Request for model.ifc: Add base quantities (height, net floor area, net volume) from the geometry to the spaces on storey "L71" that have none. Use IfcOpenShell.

First a look at what the model holds.

```python
import ifcopenshell
import ifcopenshell.util.element
import ifcopenshell.util.unit

model = ifcopenshell.open("model.ifc")
print(model.schema)
for unit_type in ("LENGTHUNIT", "AREAUNIT", "VOLUMEUNIT"):
    print(unit_type, ifcopenshell.util.unit.calculate_unit_scale(model, unit_type))
storey = next(s for s in model.by_type("IfcBuildingStorey") if s.Name == "L71")
spaces = [e for e in ifcopenshell.util.element.get_decomposition(storey) if e.is_a("IfcSpace")]
for e in sorted(spaces, key=lambda e: e.id()):
    print(e.id(), e.is_a(), e.Name, list(ifcopenshell.util.element.get_psets(e, qtos_only=True)), sep=" | ")
```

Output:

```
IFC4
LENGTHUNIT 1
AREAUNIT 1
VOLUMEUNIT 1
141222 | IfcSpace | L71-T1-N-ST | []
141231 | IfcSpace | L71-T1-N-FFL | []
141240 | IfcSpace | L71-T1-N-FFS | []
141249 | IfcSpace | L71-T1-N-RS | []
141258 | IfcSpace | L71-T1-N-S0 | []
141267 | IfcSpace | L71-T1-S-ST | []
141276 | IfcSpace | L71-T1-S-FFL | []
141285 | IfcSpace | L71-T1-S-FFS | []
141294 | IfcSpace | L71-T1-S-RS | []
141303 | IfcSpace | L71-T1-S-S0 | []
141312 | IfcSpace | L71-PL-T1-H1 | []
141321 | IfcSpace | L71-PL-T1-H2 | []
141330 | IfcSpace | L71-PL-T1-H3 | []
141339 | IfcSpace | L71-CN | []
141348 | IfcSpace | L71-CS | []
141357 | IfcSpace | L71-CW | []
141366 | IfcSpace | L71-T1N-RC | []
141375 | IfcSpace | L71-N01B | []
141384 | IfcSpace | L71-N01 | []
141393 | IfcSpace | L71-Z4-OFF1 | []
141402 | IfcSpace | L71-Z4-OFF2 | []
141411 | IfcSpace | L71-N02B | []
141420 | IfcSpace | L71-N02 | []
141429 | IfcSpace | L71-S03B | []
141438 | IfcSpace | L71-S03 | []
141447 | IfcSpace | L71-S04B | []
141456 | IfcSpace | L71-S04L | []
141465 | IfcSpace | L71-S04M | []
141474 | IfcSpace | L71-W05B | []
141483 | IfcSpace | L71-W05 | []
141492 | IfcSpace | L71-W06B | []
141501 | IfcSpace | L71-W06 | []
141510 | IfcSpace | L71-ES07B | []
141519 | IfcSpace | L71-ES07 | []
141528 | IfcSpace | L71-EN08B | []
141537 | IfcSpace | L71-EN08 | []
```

```python
import ifcopenshell
import ifcopenshell.api.pset
import ifcopenshell.geom
import ifcopenshell.util.element
import ifcopenshell.util.shape
import ifcopenshell.util.unit

model = ifcopenshell.open("model.ifc")
unit_scale = ifcopenshell.util.unit.calculate_unit_scale(model)
area_scale = ifcopenshell.util.unit.calculate_unit_scale(model, "AREAUNIT")
volume_scale = ifcopenshell.util.unit.calculate_unit_scale(model, "VOLUMEUNIT")
settings = ifcopenshell.geom.settings()

storey = next(s for s in model.by_type("IfcBuildingStorey") if s.Name == "L71")
spaces = [e for e in ifcopenshell.util.element.get_decomposition(storey) if e.is_a("IfcSpace")]

for e in sorted(spaces, key=lambda e: e.id()):
    if ifcopenshell.util.element.get_psets(e, qtos_only=True, should_inherit=False):
        continue
    # Geometry comes back in metres, in the element's own axes.
    shape = ifcopenshell.geom.create_shape(settings, e)
    values = {
        "Height": ifcopenshell.util.shape.get_z(shape.geometry) / unit_scale,
        "NetFloorArea": ifcopenshell.util.shape.get_footprint_area(shape.geometry) / area_scale,
        "NetVolume": ifcopenshell.util.shape.get_volume(shape.geometry) / volume_scale,
    }
    qto = ifcopenshell.api.pset.add_qto(model, product=e, name="Qto_SpaceBaseQuantities")
    ifcopenshell.api.pset.edit_qto(model, qto=qto, properties=values)
    print(e.id(), {k: round(v, 3) for k, v in values.items()})

model.write("model_v2.ifc")
```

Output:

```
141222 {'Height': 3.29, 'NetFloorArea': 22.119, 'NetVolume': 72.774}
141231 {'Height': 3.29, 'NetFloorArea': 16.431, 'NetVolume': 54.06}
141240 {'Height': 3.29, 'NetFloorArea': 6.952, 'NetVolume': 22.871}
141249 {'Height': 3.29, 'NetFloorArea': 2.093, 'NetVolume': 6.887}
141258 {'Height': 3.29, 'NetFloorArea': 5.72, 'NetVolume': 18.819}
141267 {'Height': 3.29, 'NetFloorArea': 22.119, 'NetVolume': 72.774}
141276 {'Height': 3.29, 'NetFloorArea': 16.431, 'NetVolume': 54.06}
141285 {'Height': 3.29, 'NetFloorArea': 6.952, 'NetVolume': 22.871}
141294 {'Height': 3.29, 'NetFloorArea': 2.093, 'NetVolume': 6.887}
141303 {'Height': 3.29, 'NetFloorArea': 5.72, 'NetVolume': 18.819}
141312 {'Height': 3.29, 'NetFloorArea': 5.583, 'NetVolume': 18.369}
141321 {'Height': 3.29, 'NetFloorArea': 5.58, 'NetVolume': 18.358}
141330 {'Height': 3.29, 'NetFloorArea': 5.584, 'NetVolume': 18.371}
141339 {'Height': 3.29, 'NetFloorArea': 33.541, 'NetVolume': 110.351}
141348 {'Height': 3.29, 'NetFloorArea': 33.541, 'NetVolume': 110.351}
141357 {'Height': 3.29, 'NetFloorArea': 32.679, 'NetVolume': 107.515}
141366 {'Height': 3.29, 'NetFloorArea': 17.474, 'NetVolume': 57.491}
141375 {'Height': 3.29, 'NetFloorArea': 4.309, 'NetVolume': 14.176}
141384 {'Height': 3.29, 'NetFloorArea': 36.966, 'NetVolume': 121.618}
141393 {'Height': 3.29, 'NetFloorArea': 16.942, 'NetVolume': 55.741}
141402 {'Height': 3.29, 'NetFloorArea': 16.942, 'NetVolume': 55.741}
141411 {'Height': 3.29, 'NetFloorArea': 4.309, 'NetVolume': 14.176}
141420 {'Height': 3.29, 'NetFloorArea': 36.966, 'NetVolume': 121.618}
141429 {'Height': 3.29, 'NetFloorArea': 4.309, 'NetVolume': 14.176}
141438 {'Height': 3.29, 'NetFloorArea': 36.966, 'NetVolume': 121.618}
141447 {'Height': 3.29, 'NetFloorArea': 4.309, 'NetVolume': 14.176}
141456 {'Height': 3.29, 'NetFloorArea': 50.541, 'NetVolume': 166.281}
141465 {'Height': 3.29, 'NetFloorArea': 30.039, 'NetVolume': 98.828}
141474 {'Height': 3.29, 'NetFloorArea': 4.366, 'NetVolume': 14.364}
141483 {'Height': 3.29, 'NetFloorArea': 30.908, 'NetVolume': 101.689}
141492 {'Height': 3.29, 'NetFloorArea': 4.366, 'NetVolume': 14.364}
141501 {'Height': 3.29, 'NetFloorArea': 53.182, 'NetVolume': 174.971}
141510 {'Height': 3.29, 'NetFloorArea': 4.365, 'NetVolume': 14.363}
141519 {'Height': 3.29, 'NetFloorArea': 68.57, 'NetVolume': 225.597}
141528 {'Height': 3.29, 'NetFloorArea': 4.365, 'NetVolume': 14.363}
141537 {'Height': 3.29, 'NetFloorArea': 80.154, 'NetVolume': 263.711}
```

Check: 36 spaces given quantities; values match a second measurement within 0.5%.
